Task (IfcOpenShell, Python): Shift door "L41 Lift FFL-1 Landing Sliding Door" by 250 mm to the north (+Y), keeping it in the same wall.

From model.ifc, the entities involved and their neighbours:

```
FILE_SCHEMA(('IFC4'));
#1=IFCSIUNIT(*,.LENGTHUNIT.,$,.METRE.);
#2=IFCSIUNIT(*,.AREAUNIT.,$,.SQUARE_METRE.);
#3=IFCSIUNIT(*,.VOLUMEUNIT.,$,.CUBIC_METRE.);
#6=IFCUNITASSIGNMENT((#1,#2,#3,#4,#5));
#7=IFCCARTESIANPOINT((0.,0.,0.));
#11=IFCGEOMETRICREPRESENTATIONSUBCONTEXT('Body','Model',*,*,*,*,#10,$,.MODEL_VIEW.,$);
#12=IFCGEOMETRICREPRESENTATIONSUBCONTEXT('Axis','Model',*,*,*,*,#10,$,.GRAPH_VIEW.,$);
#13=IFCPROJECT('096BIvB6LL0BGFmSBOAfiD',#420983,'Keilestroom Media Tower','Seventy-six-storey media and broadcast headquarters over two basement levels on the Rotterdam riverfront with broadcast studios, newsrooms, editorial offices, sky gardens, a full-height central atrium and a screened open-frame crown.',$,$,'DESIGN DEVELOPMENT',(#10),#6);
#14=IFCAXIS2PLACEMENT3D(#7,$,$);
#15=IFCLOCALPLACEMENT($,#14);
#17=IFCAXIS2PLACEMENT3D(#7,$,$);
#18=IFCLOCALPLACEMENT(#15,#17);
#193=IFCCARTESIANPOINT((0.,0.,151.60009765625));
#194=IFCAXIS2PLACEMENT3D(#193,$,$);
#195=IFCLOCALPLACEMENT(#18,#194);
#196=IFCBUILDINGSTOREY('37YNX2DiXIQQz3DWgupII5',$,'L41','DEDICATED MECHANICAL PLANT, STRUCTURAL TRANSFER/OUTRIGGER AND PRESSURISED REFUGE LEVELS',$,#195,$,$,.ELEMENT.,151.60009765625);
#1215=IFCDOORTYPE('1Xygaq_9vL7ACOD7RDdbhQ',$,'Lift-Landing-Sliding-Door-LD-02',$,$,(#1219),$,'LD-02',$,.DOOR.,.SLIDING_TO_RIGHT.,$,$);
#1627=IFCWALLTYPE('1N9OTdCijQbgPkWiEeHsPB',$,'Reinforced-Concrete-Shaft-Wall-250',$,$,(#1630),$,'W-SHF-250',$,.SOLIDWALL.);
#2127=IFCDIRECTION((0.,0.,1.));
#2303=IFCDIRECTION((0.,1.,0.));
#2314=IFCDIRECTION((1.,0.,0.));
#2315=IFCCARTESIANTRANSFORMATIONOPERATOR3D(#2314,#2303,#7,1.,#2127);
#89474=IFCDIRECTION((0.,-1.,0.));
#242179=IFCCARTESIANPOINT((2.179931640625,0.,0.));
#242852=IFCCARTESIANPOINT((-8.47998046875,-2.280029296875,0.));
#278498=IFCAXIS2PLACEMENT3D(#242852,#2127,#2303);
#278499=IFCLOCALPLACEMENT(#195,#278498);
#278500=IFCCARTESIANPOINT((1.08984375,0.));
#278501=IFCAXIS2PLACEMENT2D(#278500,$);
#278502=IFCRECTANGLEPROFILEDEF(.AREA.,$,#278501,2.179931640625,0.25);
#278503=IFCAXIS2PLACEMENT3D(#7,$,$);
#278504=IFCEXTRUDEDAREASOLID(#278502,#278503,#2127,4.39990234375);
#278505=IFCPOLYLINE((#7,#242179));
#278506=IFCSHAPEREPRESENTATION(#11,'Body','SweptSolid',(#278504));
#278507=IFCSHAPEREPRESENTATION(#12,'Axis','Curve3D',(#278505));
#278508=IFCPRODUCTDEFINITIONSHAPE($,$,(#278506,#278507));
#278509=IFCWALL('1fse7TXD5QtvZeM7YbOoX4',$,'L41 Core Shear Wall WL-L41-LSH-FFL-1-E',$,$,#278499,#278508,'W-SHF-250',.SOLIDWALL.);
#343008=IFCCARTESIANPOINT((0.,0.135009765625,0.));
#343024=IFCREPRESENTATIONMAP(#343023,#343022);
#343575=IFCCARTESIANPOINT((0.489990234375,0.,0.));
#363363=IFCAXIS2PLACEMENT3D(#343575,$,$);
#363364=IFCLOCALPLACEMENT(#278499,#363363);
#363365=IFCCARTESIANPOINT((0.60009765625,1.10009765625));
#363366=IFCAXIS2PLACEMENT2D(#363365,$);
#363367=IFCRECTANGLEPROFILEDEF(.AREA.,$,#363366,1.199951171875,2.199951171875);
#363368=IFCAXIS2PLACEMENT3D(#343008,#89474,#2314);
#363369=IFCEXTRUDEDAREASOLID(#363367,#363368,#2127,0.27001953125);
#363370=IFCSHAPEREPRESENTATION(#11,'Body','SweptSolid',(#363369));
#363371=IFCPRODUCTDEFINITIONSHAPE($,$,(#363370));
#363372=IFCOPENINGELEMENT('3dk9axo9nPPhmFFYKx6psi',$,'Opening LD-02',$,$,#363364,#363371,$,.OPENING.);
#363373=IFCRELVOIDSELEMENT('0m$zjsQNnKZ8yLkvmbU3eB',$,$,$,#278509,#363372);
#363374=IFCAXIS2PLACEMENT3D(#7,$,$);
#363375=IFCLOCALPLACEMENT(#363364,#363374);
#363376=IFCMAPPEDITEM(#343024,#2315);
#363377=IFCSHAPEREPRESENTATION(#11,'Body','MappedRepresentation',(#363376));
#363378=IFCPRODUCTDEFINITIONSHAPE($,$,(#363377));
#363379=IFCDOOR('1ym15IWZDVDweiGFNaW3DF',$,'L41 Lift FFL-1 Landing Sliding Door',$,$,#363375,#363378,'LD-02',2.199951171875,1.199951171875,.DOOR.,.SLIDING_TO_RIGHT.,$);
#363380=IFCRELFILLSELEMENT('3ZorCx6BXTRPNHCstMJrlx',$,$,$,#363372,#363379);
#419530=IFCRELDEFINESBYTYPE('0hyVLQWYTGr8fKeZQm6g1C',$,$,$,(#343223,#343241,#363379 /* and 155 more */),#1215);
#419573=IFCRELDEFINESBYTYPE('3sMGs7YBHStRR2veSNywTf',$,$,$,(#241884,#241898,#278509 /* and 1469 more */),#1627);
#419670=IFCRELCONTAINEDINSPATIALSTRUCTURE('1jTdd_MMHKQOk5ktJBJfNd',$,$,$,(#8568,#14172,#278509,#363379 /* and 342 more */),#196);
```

```python
import ifcopenshell
import ifcopenshell.api.geometry
import ifcopenshell.util.placement

model = ifcopenshell.open("model.ifc")

door = model.by_guid("1ym15IWZDVDweiGFNaW3DF")
opening = door.FillsVoids[0].RelatingOpeningElement
wall = opening.VoidsElements[0].RelatingBuildingElement

wall_matrix = ifcopenshell.util.placement.get_local_placement(wall.ObjectPlacement)
shift = wall_matrix[:3, 0] * 0.25
before = ifcopenshell.util.placement.get_local_placement(door.ObjectPlacement)[:3, 3].copy()

# The door is placed relative to its opening, so it follows when the opening moves.
matrix = ifcopenshell.util.placement.get_local_placement(opening.ObjectPlacement)
matrix[:3, 3] += shift
ifcopenshell.api.geometry.edit_object_placement(
    model, product=opening, matrix=matrix, is_si=False, should_transform_children=True
)

after = ifcopenshell.util.placement.get_local_placement(door.ObjectPlacement)[:3, 3]
print("door moved by", (after - before).round(3) + 0.0)

model.write("model-out.ifc")
```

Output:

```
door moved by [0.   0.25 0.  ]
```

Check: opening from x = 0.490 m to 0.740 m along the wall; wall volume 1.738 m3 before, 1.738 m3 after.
